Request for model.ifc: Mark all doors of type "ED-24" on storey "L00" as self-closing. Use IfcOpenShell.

First a look at what the model holds.

```python
import ifcopenshell
import ifcopenshell.util.element

model = ifcopenshell.open("model.ifc")
print(model.schema)
storey = next(s for s in model.by_type("IfcBuildingStorey") if s.Name == "L00")
doors = [e for e in ifcopenshell.util.element.get_decomposition(storey) if e.is_a("IfcDoor")]
seen = {}
for e in doors:
    element_type = ifcopenshell.util.element.get_type(e)
    key = (element_type.Name if element_type != e and element_type else None, ifcopenshell.util.element.get_pset(e, "Pset_DoorCommon", "SelfClosing"))
    seen[key] = seen.get(key, 0) + 1
for (name, value), count in sorted(seen.items(), key=str):
    print(count, "x", name, "|", value)
```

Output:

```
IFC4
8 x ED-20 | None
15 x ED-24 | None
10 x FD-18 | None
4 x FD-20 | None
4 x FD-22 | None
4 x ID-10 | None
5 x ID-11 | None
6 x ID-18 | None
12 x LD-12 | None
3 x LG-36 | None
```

```python
import ifcopenshell
import ifcopenshell.api.pset
import ifcopenshell.util.element

model = ifcopenshell.open("model.ifc")

storey = next(s for s in model.by_type("IfcBuildingStorey") if s.Name == "L00")
doors = [e for e in ifcopenshell.util.element.get_decomposition(storey) if e.is_a("IfcDoor")]

count = 0
for e in doors:
    element_type = ifcopenshell.util.element.get_type(e)
    if element_type in (None, e) or element_type.Name != "ED-24":
        continue
    # add_pset returns the element's existing set when there is one.
    pset = ifcopenshell.api.pset.add_pset(model, product=e, name="Pset_DoorCommon")
    ifcopenshell.api.pset.edit_pset(model, pset=pset, properties={"SelfClosing": True})
    count += 1

print(count, "doors updated")

model.write("model_v2.ifc")
```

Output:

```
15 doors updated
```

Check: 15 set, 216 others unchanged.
